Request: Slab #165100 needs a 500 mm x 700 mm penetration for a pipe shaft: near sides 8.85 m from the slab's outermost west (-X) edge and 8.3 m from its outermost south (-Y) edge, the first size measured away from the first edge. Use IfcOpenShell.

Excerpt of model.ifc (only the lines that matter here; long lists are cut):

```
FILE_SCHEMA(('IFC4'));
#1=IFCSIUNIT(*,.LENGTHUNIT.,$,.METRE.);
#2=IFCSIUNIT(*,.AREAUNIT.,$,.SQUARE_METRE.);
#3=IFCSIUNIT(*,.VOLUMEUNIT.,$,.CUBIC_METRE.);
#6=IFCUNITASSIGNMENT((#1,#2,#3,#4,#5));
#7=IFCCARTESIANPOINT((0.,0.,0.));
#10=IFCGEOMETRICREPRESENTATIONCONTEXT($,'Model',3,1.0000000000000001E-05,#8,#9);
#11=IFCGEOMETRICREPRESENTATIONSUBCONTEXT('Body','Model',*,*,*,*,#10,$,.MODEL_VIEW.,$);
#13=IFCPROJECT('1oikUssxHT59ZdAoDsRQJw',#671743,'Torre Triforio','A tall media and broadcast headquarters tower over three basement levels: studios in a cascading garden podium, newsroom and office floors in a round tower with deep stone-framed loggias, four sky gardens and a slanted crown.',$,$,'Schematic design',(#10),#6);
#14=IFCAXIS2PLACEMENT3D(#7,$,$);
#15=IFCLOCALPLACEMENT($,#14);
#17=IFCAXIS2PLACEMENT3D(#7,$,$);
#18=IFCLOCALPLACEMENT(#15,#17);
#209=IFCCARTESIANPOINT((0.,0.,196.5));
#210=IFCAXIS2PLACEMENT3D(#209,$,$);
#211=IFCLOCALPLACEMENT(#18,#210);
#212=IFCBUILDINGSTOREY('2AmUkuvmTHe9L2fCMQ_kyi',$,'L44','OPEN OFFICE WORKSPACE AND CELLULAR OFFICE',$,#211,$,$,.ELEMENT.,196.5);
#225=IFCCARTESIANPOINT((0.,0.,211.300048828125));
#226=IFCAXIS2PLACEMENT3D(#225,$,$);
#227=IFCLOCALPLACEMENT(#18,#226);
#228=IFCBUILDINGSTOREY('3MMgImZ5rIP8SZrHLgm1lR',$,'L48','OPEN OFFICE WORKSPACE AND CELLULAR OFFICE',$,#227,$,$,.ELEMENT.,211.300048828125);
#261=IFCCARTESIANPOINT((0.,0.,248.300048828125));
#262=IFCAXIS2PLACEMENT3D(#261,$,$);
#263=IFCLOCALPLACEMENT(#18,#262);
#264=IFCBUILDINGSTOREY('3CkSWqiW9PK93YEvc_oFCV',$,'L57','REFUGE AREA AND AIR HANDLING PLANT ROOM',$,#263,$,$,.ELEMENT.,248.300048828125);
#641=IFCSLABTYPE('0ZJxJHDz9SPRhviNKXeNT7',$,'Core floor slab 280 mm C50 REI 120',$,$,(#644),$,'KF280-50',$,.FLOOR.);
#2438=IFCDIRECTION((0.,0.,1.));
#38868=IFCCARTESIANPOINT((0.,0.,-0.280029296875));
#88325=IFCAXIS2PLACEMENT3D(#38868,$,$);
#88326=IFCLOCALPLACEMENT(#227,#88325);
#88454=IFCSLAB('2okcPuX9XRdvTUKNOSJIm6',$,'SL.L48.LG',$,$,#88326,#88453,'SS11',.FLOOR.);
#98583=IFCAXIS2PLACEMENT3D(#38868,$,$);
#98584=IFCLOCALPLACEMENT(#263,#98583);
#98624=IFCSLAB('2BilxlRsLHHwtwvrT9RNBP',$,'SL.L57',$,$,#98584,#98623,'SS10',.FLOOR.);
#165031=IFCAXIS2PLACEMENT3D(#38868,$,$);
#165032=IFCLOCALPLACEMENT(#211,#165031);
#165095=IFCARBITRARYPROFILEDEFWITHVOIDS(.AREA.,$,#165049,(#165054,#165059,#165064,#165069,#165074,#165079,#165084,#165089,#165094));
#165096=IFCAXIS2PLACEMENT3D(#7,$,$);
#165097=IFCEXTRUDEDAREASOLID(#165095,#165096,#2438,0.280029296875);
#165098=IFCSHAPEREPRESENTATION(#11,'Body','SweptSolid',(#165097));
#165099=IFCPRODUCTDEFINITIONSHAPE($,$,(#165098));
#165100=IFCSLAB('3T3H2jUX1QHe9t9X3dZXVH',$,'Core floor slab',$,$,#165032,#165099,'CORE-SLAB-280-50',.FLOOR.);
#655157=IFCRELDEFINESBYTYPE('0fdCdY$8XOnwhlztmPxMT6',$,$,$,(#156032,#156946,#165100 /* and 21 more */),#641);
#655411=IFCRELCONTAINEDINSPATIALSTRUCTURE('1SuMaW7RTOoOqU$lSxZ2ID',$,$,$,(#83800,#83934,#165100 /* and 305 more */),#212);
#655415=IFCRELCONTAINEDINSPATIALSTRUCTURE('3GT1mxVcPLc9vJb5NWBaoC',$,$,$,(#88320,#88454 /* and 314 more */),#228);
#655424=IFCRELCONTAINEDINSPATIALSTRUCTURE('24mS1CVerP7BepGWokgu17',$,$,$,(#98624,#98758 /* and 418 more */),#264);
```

```python
import numpy as np
import ifcopenshell
import ifcopenshell.api.feature
import ifcopenshell.api.geometry
import ifcopenshell.api.root
import ifcopenshell.geom
import ifcopenshell.util.placement
import ifcopenshell.util.representation
import ifcopenshell.util.shape
import ifcopenshell.util.unit

model = ifcopenshell.open("model.ifc")
unit_scale = ifcopenshell.util.unit.calculate_unit_scale(model)
settings = ifcopenshell.geom.settings()


def volume(element):
    """Net volume in cubic metres, openings subtracted."""
    shape = ifcopenshell.geom.create_shape(settings, element)
    return ifcopenshell.util.shape.get_volume(shape.geometry)


slab = model.by_guid("3T3H2jUX1QHe9t9X3dZXVH")
before = volume(slab)

# Extent in the slab's own axes, in metres. The edges named are its -X and -Y sides.
slab_shape = ifcopenshell.geom.create_shape(settings, slab)
vertices = ifcopenshell.util.shape.get_vertices(slab_shape.geometry)
x_min, y_min, bottom = vertices.min(axis=0)
top = vertices[:, 2].max()

opening = ifcopenshell.api.root.create_entity(model, ifc_class="IfcOpeningElement", name="Pipe shaft opening", predefined_type="OPENING")
context = ifcopenshell.util.representation.get_context(model, "Model", "Body", "MODEL_VIEW")
width, depth = 0.5, 0.7
outline = [(0.0, 0.0), (width, 0.0), (width, depth), (0.0, depth), (0.0, 0.0)]
# Overshoot both faces by 50 mm so the cut is clean.
shape = ifcopenshell.api.geometry.add_slab_representation(
    model, context=context, depth=top - bottom + 0.1, polyline=outline
)
ifcopenshell.api.geometry.assign_representation(model, product=opening, representation=shape)

matrix = ifcopenshell.util.placement.get_local_placement(slab.ObjectPlacement)
matrix[:, 3] = matrix @ np.append(np.array([x_min + 8.85, y_min + 8.3, bottom - 0.05]) / unit_scale, 1.0)
ifcopenshell.api.geometry.edit_object_placement(model, product=opening, matrix=matrix, is_si=False)
ifcopenshell.api.feature.add_feature(model, feature=opening, element=slab)

after = volume(slab)

print(f"slab volume {before:.3f} -> {after:.3f} m3")

model.write("model_rev.ifc")
```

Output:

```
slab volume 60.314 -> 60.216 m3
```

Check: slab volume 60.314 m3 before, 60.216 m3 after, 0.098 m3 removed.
